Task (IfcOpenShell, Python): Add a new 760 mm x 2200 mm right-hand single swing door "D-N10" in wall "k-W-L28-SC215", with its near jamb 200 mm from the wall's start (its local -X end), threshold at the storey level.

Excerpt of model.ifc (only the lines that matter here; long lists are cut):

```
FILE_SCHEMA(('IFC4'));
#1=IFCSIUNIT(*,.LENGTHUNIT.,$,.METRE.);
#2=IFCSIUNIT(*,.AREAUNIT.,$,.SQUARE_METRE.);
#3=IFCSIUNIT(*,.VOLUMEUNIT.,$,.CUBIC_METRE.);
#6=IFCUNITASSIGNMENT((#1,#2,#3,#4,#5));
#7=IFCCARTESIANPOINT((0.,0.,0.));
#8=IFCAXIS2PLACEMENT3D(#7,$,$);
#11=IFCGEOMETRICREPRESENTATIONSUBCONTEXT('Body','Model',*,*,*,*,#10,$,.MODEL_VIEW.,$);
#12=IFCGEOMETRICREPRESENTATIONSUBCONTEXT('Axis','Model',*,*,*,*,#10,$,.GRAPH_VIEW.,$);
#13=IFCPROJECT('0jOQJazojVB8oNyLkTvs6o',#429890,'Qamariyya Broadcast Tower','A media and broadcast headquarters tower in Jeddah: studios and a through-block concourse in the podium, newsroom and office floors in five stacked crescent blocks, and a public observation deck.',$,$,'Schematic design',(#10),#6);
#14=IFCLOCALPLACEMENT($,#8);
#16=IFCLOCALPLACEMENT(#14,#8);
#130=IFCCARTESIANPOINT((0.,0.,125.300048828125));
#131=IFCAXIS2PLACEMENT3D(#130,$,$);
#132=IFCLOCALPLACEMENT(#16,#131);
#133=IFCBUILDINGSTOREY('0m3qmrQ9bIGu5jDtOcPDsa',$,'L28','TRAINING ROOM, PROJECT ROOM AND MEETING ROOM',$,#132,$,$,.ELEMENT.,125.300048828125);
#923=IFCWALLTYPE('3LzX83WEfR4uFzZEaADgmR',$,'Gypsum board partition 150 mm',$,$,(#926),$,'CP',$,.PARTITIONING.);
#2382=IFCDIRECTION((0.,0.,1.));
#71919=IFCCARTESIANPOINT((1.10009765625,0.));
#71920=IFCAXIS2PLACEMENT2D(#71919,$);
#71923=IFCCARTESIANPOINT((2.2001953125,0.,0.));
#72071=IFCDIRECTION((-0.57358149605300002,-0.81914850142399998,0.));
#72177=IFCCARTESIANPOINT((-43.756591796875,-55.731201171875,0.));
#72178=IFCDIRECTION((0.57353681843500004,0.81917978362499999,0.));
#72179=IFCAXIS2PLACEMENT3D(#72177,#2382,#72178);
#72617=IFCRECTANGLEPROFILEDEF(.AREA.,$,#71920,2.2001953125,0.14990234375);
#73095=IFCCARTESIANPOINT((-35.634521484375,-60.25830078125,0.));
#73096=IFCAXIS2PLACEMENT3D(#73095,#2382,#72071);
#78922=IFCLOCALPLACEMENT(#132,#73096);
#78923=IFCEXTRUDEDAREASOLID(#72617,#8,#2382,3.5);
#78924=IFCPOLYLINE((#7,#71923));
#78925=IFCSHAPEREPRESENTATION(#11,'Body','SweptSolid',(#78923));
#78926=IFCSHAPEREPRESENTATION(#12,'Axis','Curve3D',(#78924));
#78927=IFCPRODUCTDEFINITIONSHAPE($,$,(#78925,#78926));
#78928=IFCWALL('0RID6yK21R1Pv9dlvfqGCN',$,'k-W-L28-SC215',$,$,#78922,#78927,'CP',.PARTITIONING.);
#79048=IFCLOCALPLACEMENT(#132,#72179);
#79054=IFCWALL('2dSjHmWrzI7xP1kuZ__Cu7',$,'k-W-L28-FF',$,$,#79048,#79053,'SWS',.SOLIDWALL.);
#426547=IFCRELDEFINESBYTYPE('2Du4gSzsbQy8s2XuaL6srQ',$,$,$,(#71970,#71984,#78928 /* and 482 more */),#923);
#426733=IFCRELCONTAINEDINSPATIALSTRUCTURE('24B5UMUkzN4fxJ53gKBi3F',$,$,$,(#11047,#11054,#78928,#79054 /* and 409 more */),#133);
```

```python
import numpy as np
import ifcopenshell
import ifcopenshell.api.feature
import ifcopenshell.api.geometry
import ifcopenshell.api.root
import ifcopenshell.api.spatial
import ifcopenshell.geom
import ifcopenshell.util.element
import ifcopenshell.util.placement
import ifcopenshell.util.representation
import ifcopenshell.util.shape
import ifcopenshell.util.unit

model = ifcopenshell.open("model.ifc")
unit_scale = ifcopenshell.util.unit.calculate_unit_scale(model)
settings = ifcopenshell.geom.settings()


def volume(element):
    """Net volume in cubic metres, openings subtracted."""
    shape = ifcopenshell.geom.create_shape(settings, element)
    return ifcopenshell.util.shape.get_volume(shape.geometry)


wall = model.by_id(78928)
storey = ifcopenshell.util.element.get_container(wall, ifc_class="IfcBuildingStorey")
context = ifcopenshell.util.representation.get_context(model, "Model", "Body", "MODEL_VIEW")
before = volume(wall)

width, height, from_end, sill = 0.76, 2.2, 0.2, 0.0  # metres

# The wall runs along its own X axis, and the end named is its -X end.
wall_shape = ifcopenshell.geom.create_shape(settings, wall)
x, y, z = ifcopenshell.util.shape.get_vertices(wall_shape.geometry).T
start = x.min() + from_end
face, thickness = float(y.min()), float(y.max() - y.min())
wall_matrix = ifcopenshell.util.placement.get_local_placement(wall.ObjectPlacement)
level = ifcopenshell.util.placement.get_local_placement(storey.ObjectPlacement)[2, 3]


def in_wall(x, y):
    """Placement at x, y metres in the wall's axes, at sill height."""
    matrix = wall_matrix.copy()
    matrix[:, 3] = wall_matrix @ np.array([x / unit_scale, y / unit_scale, 0.0, 1.0])
    matrix[2, 3] = level + sill / unit_scale
    return matrix


# Opening: a box that overshoots both wall faces by 50 mm.
opening = ifcopenshell.api.root.create_entity(model, ifc_class="IfcOpeningElement", predefined_type="OPENING")
box = ifcopenshell.api.geometry.add_wall_representation(
    model, context=context, length=width, height=height, thickness=thickness + 0.1
)
ifcopenshell.api.geometry.assign_representation(model, product=opening, representation=box)
ifcopenshell.api.geometry.edit_object_placement(model, product=opening, matrix=in_wall(start, face - 0.05), is_si=False)
ifcopenshell.api.feature.add_feature(model, feature=opening, element=wall)

door = ifcopenshell.api.root.create_entity(model, ifc_class="IfcDoor", name="D-N10", predefined_type="DOOR")
door.OverallWidth, door.OverallHeight = width / unit_scale, height / unit_scale
door.OperationType = "SINGLE_SWING_RIGHT"
body = ifcopenshell.api.geometry.add_door_representation(
    model,
    context=context,
    overall_width=door.OverallWidth,
    overall_height=door.OverallHeight,
    operation_type="SINGLE_SWING_RIGHT",
    lining_properties={"LiningDepth": thickness / unit_scale, "ThresholdDepth": thickness / unit_scale},
)
ifcopenshell.api.geometry.assign_representation(model, product=door, representation=body)
ifcopenshell.api.spatial.assign_container(model, products=[door], relating_structure=storey)
ifcopenshell.api.feature.add_filling(model, opening=opening, element=door)

# The lining spans the wall, so the door starts at the wall face.
ifcopenshell.api.geometry.edit_object_placement(model, product=door, matrix=in_wall(start, face), is_si=False)

after = volume(wall)

print(f"wall volume {before:.3f} -> {after:.3f} m3")

model.write("model_v2.ifc")
```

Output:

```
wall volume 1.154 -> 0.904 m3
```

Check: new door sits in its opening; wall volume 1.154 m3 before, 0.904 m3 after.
